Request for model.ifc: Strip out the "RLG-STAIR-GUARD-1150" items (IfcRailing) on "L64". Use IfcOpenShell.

First a look at what the model holds.

```python
import ifcopenshell
import ifcopenshell.util.element

model = ifcopenshell.open("model.ifc")
print(model.schema)
storey = next(s for s in model.by_type("IfcBuildingStorey") if s.Name == "L64")
railings = [e for e in ifcopenshell.util.element.get_decomposition(storey) if e.is_a("IfcRailing")]
seen = {}
for e in railings:
    element_type = ifcopenshell.util.element.get_type(e)
    name = element_type.Name if element_type not in (None, e) else None
    seen[name] = seen.get(name, 0) + 1
for name, count in sorted(seen.items(), key=str):
    print(count, "x", name)
```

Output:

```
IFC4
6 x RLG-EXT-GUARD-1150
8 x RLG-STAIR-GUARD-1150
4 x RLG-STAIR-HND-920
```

```python
import ifcopenshell
import ifcopenshell.api.root
import ifcopenshell.util.element

model = ifcopenshell.open("model.ifc")

storey = next(s for s in model.by_type("IfcBuildingStorey") if s.Name == "L64")
railings = [e for e in ifcopenshell.util.element.get_decomposition(storey) if e.is_a("IfcRailing")]
targets = [e for e in railings if (t := ifcopenshell.util.element.get_type(e)) not in (None, e) and t.Name == "RLG-STAIR-GUARD-1150"]

for e in targets:
    ifcopenshell.api.root.remove_product(model, product=e)
print(len(targets), "removed")

model.write("model_v2.ifc")
```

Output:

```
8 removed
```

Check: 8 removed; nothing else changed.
